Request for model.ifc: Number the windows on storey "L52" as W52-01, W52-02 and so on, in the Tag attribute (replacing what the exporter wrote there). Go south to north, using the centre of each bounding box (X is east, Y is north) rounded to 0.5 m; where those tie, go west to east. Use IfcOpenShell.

First a look at what the model holds.

```python
import ifcopenshell
import ifcopenshell.util.element
import ifcopenshell.util.placement

model = ifcopenshell.open("model.ifc")
print(model.schema)
storey = next(s for s in model.by_type("IfcBuildingStorey") if s.Name == "L52")
windows = [e for e in ifcopenshell.util.element.get_decomposition(storey) if e.is_a("IfcWindow")]
for e in sorted(windows, key=lambda e: e.id()):
    origin = ifcopenshell.util.placement.get_local_placement(e.ObjectPlacement)[:3, 3]
    print(e.id(), e.Tag, e.Name, origin.round(2) + 0.0, sep=" | ")
```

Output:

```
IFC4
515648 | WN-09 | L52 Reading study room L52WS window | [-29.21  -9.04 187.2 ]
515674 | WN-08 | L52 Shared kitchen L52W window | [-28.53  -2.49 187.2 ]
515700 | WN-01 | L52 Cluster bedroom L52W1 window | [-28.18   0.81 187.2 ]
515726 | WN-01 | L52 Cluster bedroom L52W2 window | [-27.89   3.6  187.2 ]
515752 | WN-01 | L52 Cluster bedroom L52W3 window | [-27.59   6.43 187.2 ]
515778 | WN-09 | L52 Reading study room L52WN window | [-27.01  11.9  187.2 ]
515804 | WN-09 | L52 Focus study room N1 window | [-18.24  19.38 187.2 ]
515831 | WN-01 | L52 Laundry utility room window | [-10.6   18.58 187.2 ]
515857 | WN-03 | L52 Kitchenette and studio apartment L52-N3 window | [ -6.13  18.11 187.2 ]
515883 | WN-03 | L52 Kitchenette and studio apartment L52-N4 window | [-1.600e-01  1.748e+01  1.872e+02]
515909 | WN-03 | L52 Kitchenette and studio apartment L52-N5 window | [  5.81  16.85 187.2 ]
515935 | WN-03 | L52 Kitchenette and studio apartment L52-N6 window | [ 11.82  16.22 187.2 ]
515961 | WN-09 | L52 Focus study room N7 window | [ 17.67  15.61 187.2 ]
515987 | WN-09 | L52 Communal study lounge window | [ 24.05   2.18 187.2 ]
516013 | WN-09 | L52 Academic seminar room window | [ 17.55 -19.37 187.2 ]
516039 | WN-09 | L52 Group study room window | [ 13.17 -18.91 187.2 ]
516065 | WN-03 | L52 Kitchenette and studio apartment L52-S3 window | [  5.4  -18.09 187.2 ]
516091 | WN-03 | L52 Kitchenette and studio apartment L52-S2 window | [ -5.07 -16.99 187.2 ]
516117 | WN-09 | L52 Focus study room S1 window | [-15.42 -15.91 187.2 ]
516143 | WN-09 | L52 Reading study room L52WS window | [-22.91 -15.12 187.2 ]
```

```python
import ifcopenshell
import ifcopenshell.geom
import ifcopenshell.util.element
import ifcopenshell.util.shape

model = ifcopenshell.open("model.ifc")
settings = ifcopenshell.geom.settings()
settings.set("use-world-coords", True)


def centre(element):
    shape = ifcopenshell.geom.create_shape(settings, element)
    return ifcopenshell.util.shape.get_bbox_centroid(shape.geometry)


storey = next(s for s in model.by_type("IfcBuildingStorey") if s.Name == "L52")
windows = [e for e in ifcopenshell.util.element.get_decomposition(storey) if e.is_a("IfcWindow")]

# Insertion points can sit at a corner or the storey origin, so sort by the geometry (in metres).
centres = {e: centre(e) for e in windows}
windows.sort(key=lambda e: (round(centres[e][1] / 0.5), centres[e][0]))

for i, e in enumerate(windows, start=1):
    number = f"W52-{i:02d}"
    e.Tag = number
    print(e.id(), number)

model.write("model_rev.ifc")
```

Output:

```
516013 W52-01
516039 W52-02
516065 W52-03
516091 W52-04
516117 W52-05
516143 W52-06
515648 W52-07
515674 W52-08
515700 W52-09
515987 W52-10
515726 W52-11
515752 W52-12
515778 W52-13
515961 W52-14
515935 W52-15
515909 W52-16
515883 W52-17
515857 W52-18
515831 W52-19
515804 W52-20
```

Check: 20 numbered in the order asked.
